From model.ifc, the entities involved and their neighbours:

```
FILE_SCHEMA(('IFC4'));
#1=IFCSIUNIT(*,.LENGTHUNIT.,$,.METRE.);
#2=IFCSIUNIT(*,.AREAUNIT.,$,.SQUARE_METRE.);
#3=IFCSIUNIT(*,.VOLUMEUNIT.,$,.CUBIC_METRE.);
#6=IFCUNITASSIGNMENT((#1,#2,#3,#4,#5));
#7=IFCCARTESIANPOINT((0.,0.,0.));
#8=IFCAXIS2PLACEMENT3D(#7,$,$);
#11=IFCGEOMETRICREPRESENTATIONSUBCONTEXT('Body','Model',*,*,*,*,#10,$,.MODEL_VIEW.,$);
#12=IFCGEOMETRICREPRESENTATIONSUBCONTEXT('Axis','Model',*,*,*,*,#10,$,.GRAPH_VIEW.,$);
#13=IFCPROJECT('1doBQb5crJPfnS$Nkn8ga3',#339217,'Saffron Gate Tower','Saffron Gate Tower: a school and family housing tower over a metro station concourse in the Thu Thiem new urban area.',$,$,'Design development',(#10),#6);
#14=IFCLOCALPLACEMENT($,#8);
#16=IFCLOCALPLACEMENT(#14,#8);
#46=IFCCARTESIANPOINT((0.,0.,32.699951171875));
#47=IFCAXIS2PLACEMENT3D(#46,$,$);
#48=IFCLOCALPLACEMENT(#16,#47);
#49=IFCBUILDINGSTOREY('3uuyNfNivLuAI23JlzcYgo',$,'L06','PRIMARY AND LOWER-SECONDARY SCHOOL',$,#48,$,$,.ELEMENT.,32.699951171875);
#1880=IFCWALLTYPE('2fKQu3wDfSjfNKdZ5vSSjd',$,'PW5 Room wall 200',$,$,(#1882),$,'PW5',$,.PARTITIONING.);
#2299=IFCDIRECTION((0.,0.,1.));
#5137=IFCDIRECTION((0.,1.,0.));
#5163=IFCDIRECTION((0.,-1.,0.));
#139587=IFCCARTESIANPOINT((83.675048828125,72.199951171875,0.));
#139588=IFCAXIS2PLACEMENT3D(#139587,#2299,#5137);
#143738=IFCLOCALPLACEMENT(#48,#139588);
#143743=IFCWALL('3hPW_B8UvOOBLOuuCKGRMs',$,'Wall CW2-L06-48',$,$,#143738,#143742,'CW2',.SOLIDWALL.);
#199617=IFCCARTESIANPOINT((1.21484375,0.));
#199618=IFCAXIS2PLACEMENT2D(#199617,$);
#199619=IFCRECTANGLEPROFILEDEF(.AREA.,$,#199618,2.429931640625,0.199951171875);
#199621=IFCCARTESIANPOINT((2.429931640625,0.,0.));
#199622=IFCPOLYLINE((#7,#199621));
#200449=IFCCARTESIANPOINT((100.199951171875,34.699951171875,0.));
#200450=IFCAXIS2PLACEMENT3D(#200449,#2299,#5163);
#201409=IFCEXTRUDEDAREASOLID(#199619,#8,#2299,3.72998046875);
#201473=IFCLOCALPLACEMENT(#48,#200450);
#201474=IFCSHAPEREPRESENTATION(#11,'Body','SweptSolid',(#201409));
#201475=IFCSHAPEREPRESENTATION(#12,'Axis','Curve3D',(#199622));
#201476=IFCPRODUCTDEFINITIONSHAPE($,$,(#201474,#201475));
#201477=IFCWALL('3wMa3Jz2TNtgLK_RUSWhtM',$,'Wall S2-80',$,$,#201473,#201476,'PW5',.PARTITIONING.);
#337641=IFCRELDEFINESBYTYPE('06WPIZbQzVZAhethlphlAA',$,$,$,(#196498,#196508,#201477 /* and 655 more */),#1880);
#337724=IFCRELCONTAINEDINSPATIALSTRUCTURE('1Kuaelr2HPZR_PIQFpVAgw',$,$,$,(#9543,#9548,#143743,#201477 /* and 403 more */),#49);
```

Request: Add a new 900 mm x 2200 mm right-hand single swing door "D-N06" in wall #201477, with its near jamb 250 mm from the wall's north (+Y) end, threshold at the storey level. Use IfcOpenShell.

```python
import numpy as np
import ifcopenshell
import ifcopenshell.api.feature
import ifcopenshell.api.geometry
import ifcopenshell.api.root
import ifcopenshell.api.spatial
import ifcopenshell.geom
import ifcopenshell.util.element
import ifcopenshell.util.placement
import ifcopenshell.util.representation
import ifcopenshell.util.shape
import ifcopenshell.util.unit

model = ifcopenshell.open("model.ifc")
unit_scale = ifcopenshell.util.unit.calculate_unit_scale(model)
settings = ifcopenshell.geom.settings()


def volume(element):
    """Net volume in cubic metres, openings subtracted."""
    shape = ifcopenshell.geom.create_shape(settings, element)
    return ifcopenshell.util.shape.get_volume(shape.geometry)


wall = model.by_guid("3wMa3Jz2TNtgLK_RUSWhtM")
storey = ifcopenshell.util.element.get_container(wall, ifc_class="IfcBuildingStorey")
context = ifcopenshell.util.representation.get_context(model, "Model", "Body", "MODEL_VIEW")
before = volume(wall)

width, height, from_end, sill = 0.9, 2.2, 0.25, 0.0  # metres

# The wall runs along its own X axis, and the end named is its -X end.
wall_shape = ifcopenshell.geom.create_shape(settings, wall)
x, y, z = ifcopenshell.util.shape.get_vertices(wall_shape.geometry).T
start = x.min() + from_end
face, thickness = float(y.min()), float(y.max() - y.min())
wall_matrix = ifcopenshell.util.placement.get_local_placement(wall.ObjectPlacement)
level = ifcopenshell.util.placement.get_local_placement(storey.ObjectPlacement)[2, 3]


def in_wall(x, y):
    """Placement at x, y metres in the wall's axes, at sill height."""
    matrix = wall_matrix.copy()
    matrix[:, 3] = wall_matrix @ np.array([x / unit_scale, y / unit_scale, 0.0, 1.0])
    matrix[2, 3] = level + sill / unit_scale
    return matrix


# Opening: a box that overshoots both wall faces by 50 mm.
opening = ifcopenshell.api.root.create_entity(model, ifc_class="IfcOpeningElement", predefined_type="OPENING")
box = ifcopenshell.api.geometry.add_wall_representation(
    model, context=context, length=width, height=height, thickness=thickness + 0.1
)
ifcopenshell.api.geometry.assign_representation(model, product=opening, representation=box)
ifcopenshell.api.geometry.edit_object_placement(model, product=opening, matrix=in_wall(start, face - 0.05), is_si=False)
ifcopenshell.api.feature.add_feature(model, feature=opening, element=wall)

door = ifcopenshell.api.root.create_entity(model, ifc_class="IfcDoor", name="D-N06", predefined_type="DOOR")
door.OverallWidth, door.OverallHeight = width / unit_scale, height / unit_scale
door.OperationType = "SINGLE_SWING_RIGHT"
body = ifcopenshell.api.geometry.add_door_representation(
    model,
    context=context,
    overall_width=door.OverallWidth,
    overall_height=door.OverallHeight,
    operation_type="SINGLE_SWING_RIGHT",
    lining_properties={"LiningDepth": thickness / unit_scale, "ThresholdDepth": thickness / unit_scale},
)
ifcopenshell.api.geometry.assign_representation(model, product=door, representation=body)
ifcopenshell.api.spatial.assign_container(model, products=[door], relating_structure=storey)
ifcopenshell.api.feature.add_filling(model, opening=opening, element=door)

# The lining spans the wall, so the door starts at the wall face.
ifcopenshell.api.geometry.edit_object_placement(model, product=door, matrix=in_wall(start, face), is_si=False)

after = volume(wall)

print(f"wall volume {before:.3f} -> {after:.3f} m3")

model.write("model_updated.ifc")
```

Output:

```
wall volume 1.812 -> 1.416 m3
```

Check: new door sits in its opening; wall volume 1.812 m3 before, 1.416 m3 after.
